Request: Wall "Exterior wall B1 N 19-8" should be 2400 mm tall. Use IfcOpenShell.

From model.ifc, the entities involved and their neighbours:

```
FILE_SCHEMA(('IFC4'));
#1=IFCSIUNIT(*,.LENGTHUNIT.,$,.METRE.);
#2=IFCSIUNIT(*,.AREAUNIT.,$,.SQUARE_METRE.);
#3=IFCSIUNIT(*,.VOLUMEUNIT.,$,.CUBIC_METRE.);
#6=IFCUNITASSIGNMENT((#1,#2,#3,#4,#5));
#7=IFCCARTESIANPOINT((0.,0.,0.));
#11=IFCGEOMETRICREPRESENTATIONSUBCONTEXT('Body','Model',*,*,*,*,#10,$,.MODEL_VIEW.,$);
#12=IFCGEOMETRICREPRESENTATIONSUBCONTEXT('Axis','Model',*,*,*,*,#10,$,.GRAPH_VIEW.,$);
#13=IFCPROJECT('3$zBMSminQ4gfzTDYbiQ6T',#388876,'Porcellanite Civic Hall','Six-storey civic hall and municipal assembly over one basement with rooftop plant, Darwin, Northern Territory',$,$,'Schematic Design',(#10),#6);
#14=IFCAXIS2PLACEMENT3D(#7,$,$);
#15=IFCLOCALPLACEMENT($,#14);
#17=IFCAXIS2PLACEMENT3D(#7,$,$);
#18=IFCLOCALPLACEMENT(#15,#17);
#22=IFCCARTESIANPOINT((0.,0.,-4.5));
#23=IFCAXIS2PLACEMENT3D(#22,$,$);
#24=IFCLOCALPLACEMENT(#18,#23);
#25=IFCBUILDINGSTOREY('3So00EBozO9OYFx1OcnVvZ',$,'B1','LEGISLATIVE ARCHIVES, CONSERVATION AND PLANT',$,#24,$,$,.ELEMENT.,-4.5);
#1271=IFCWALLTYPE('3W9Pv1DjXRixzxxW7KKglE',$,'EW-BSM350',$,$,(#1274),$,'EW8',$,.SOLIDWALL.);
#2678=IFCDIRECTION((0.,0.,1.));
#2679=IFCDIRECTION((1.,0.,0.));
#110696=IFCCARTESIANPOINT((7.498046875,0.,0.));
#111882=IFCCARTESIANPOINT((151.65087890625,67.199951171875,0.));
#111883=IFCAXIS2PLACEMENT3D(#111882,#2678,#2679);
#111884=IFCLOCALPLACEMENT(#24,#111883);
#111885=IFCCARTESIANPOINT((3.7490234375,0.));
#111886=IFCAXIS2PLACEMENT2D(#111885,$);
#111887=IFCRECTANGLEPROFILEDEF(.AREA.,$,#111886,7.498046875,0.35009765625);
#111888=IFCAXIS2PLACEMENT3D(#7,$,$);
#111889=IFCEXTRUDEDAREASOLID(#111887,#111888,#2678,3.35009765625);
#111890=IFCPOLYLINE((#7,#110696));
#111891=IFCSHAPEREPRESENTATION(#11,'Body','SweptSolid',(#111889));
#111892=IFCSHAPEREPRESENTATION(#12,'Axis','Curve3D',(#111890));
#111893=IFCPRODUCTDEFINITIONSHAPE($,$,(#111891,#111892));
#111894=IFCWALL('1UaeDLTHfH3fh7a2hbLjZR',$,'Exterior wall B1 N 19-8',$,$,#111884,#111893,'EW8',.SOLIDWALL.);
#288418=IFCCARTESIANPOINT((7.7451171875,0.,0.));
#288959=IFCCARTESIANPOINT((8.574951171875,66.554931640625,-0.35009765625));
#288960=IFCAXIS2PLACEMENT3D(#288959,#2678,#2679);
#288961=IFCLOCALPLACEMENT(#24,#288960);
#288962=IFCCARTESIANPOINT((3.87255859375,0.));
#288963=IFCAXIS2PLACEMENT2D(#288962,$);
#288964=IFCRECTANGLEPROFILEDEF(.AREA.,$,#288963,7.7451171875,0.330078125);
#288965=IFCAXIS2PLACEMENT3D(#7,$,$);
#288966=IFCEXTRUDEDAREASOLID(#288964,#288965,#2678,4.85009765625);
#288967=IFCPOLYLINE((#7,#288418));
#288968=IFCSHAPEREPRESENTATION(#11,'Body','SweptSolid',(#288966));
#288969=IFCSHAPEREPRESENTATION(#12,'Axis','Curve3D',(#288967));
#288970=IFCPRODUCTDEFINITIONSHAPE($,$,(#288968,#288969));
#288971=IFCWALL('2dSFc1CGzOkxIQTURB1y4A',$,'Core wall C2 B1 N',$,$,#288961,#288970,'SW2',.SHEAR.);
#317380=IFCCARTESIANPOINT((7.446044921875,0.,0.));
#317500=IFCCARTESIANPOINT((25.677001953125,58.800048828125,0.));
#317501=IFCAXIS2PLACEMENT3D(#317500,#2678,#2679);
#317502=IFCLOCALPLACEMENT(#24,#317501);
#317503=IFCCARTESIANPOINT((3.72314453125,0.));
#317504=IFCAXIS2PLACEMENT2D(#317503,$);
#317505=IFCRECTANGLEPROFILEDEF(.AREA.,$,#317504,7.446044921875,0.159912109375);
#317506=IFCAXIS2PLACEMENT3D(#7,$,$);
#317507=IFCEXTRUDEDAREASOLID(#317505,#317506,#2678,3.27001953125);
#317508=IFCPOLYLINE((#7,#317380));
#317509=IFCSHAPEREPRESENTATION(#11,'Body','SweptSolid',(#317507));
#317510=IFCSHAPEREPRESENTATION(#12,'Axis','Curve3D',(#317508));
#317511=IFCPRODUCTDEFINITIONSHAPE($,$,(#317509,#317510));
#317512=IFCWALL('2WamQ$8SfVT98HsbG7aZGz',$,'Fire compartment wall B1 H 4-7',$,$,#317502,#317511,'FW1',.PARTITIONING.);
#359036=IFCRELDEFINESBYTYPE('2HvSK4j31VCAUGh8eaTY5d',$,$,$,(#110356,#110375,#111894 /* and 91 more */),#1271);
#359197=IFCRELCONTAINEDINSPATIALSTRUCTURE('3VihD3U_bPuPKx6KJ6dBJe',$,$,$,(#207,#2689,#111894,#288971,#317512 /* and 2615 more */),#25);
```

```python
import ifcopenshell
import ifcopenshell.geom
import ifcopenshell.util.representation
import ifcopenshell.util.shape
import ifcopenshell.util.unit

model = ifcopenshell.open("model.ifc")
unit_scale = ifcopenshell.util.unit.calculate_unit_scale(model)
settings = ifcopenshell.geom.settings()


def volume(element):
    """Net volume in cubic metres, openings subtracted."""
    shape = ifcopenshell.geom.create_shape(settings, element)
    return ifcopenshell.util.shape.get_volume(shape.geometry)


wall = model.by_id(111894)
before = volume(wall)

body = ifcopenshell.util.representation.get_representation(wall, "Model", "Body")
solid = body.Items[0]
old_height = solid.Depth
solid.Depth = 2.4 / unit_scale
after = volume(wall)

print(f"height {old_height:g} -> {solid.Depth:g}, volume {before:.3f} -> {after:.3f} m3")

model.write("model-out.ifc")
```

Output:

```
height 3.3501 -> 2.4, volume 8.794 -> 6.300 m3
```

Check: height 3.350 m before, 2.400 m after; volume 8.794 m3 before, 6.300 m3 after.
